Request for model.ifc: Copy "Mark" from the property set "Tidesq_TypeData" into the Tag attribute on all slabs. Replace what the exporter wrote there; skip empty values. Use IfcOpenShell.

First a look at what the model holds.

```python
import ifcopenshell
import ifcopenshell.util.element

model = ifcopenshell.open("model.ifc")
print(model.schema)
slabs = model.by_type("IfcSlab")
print(len(slabs), "slabs")
for e in slabs[:8]:
    source = ifcopenshell.util.element.get_pset(e, "Tidesq_TypeData", "Mark")
    target = e.Tag
    print(e.id(), repr(source), repr(target), sep=" | ")
```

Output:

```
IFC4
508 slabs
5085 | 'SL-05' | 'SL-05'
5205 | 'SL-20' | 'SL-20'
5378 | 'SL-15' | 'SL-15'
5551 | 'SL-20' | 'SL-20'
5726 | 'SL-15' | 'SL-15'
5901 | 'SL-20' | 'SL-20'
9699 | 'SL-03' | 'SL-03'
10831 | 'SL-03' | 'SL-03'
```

```python
import ifcopenshell
import ifcopenshell.util.element

model = ifcopenshell.open("model.ifc")

count = 0
for e in model.by_type("IfcSlab"):
    value = ifcopenshell.util.element.get_pset(e, "Tidesq_TypeData", "Mark")
    current = e.Tag
    if not value or not value.strip() or current == value:
        continue
    e.Tag = value
    count += 1

print(count, "slabs updated")

model.write("model_v2.ifc")
```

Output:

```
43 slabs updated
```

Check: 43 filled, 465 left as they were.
